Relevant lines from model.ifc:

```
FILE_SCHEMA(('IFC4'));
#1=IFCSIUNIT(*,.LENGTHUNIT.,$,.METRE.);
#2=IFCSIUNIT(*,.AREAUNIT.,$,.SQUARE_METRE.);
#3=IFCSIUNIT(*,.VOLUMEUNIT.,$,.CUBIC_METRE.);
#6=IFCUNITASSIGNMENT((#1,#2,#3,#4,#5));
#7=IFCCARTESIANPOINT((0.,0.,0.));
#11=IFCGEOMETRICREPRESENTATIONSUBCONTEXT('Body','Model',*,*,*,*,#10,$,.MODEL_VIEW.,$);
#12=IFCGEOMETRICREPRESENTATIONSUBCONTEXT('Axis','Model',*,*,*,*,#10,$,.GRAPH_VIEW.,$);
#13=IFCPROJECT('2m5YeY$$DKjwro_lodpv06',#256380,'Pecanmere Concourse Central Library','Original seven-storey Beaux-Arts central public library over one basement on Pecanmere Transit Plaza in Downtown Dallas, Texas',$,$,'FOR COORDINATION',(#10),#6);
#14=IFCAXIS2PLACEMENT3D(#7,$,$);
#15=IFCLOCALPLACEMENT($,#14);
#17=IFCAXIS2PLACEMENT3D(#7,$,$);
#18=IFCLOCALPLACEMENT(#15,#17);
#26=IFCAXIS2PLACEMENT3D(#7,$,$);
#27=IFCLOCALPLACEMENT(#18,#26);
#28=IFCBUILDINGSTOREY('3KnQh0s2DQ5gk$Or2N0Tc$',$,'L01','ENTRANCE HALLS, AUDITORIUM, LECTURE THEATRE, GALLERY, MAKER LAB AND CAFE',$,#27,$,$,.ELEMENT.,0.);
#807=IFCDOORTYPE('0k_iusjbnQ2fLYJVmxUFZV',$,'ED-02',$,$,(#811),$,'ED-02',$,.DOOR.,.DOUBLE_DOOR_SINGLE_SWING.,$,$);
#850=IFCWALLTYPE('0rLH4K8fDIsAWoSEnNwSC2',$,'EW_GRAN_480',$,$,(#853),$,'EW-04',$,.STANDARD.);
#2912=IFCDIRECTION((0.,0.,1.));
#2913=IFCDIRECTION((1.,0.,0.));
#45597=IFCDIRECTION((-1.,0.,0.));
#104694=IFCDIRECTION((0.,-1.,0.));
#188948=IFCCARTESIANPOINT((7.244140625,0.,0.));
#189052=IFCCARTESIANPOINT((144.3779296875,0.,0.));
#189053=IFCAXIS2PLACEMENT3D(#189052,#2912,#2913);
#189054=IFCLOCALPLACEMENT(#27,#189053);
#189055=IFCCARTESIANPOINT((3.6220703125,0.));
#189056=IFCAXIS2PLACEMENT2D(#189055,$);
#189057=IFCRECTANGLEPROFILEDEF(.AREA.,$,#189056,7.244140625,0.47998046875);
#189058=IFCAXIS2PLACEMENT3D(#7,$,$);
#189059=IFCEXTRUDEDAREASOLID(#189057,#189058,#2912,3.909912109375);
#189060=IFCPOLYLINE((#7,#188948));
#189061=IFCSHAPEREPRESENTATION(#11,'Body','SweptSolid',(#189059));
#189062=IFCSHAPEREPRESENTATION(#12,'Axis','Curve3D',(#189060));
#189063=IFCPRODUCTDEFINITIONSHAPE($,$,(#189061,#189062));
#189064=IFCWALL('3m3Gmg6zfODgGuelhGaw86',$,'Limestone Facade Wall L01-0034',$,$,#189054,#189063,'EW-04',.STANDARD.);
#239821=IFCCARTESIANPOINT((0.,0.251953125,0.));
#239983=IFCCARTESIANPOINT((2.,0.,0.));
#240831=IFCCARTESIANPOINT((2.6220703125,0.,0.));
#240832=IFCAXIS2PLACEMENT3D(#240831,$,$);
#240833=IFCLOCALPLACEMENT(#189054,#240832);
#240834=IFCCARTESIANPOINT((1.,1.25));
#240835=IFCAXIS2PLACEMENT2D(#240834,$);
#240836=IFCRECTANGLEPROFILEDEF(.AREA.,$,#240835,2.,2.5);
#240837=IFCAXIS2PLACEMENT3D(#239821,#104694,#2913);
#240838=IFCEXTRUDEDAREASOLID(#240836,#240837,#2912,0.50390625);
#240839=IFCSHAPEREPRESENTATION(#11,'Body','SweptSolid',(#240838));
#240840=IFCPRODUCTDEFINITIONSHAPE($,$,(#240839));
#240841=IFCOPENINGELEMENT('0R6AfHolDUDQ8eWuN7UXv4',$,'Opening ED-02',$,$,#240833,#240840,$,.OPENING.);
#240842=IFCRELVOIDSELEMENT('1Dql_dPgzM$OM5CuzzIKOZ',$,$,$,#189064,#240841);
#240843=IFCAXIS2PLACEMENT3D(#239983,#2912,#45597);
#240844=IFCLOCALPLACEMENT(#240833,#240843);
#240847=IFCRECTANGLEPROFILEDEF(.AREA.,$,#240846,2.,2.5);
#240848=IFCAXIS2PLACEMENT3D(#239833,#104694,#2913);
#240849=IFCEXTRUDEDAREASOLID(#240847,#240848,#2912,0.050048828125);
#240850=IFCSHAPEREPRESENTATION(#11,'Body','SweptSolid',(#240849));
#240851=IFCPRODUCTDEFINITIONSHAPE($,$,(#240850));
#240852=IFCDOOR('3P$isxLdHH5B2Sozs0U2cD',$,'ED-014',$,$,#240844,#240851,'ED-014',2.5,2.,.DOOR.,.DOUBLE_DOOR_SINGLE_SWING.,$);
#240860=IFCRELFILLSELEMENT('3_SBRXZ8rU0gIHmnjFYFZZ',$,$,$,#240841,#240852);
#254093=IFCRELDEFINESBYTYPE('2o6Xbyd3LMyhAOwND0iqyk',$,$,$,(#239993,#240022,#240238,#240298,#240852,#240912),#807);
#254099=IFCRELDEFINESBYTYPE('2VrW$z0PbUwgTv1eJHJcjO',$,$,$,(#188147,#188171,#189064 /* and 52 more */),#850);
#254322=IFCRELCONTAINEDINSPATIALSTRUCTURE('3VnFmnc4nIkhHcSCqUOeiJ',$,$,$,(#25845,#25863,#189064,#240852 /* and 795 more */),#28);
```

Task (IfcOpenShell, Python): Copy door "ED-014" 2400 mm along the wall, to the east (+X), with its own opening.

```python
import ifcopenshell
import ifcopenshell.api.feature
import ifcopenshell.api.geometry
import ifcopenshell.api.root
import ifcopenshell.geom
import ifcopenshell.util.element
import ifcopenshell.util.placement
import ifcopenshell.util.shape

model = ifcopenshell.open("model.ifc")
settings = ifcopenshell.geom.settings()


def volume(element):
    """Net volume in cubic metres, openings subtracted."""
    shape = ifcopenshell.geom.create_shape(settings, element)
    return ifcopenshell.util.shape.get_volume(shape.geometry)


door = model.by_guid("3P$isxLdHH5B2Sozs0U2cD")
opening = door.FillsVoids[0].RelatingOpeningElement
wall = opening.VoidsElements[0].RelatingBuildingElement
before = volume(wall)
shift = ifcopenshell.util.placement.get_local_placement(wall.ObjectPlacement)[:3, 0] * 2.4

# copy_class copies the void relationship, type, container and properties, but no geometry.
new_opening = ifcopenshell.api.root.copy_class(model, product=opening)
new_opening.Representation = ifcopenshell.util.element.copy_deep(
    model, opening.Representation, exclude=["IfcGeometricRepresentationContext", "IfcRepresentationMap"]
)
new_door = ifcopenshell.api.root.copy_class(model, product=door)
new_door.Representation = ifcopenshell.util.element.copy_deep(
    model, door.Representation, exclude=["IfcGeometricRepresentationContext", "IfcRepresentationMap"]
)
new_door.Tag = None
ifcopenshell.api.feature.add_filling(model, opening=new_opening, element=new_door)

for old, new in ((opening, new_opening), (door, new_door)):
    matrix = ifcopenshell.util.placement.get_local_placement(old.ObjectPlacement)
    matrix[:3, 3] += shift
    ifcopenshell.api.geometry.edit_object_placement(model, product=new, matrix=matrix, is_si=False)

after = volume(wall)

print(f"wall volume {before:.3f} -> {after:.3f} m3")

model.write("model-out.ifc")
```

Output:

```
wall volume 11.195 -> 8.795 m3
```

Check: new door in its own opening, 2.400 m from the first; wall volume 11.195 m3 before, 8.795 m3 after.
